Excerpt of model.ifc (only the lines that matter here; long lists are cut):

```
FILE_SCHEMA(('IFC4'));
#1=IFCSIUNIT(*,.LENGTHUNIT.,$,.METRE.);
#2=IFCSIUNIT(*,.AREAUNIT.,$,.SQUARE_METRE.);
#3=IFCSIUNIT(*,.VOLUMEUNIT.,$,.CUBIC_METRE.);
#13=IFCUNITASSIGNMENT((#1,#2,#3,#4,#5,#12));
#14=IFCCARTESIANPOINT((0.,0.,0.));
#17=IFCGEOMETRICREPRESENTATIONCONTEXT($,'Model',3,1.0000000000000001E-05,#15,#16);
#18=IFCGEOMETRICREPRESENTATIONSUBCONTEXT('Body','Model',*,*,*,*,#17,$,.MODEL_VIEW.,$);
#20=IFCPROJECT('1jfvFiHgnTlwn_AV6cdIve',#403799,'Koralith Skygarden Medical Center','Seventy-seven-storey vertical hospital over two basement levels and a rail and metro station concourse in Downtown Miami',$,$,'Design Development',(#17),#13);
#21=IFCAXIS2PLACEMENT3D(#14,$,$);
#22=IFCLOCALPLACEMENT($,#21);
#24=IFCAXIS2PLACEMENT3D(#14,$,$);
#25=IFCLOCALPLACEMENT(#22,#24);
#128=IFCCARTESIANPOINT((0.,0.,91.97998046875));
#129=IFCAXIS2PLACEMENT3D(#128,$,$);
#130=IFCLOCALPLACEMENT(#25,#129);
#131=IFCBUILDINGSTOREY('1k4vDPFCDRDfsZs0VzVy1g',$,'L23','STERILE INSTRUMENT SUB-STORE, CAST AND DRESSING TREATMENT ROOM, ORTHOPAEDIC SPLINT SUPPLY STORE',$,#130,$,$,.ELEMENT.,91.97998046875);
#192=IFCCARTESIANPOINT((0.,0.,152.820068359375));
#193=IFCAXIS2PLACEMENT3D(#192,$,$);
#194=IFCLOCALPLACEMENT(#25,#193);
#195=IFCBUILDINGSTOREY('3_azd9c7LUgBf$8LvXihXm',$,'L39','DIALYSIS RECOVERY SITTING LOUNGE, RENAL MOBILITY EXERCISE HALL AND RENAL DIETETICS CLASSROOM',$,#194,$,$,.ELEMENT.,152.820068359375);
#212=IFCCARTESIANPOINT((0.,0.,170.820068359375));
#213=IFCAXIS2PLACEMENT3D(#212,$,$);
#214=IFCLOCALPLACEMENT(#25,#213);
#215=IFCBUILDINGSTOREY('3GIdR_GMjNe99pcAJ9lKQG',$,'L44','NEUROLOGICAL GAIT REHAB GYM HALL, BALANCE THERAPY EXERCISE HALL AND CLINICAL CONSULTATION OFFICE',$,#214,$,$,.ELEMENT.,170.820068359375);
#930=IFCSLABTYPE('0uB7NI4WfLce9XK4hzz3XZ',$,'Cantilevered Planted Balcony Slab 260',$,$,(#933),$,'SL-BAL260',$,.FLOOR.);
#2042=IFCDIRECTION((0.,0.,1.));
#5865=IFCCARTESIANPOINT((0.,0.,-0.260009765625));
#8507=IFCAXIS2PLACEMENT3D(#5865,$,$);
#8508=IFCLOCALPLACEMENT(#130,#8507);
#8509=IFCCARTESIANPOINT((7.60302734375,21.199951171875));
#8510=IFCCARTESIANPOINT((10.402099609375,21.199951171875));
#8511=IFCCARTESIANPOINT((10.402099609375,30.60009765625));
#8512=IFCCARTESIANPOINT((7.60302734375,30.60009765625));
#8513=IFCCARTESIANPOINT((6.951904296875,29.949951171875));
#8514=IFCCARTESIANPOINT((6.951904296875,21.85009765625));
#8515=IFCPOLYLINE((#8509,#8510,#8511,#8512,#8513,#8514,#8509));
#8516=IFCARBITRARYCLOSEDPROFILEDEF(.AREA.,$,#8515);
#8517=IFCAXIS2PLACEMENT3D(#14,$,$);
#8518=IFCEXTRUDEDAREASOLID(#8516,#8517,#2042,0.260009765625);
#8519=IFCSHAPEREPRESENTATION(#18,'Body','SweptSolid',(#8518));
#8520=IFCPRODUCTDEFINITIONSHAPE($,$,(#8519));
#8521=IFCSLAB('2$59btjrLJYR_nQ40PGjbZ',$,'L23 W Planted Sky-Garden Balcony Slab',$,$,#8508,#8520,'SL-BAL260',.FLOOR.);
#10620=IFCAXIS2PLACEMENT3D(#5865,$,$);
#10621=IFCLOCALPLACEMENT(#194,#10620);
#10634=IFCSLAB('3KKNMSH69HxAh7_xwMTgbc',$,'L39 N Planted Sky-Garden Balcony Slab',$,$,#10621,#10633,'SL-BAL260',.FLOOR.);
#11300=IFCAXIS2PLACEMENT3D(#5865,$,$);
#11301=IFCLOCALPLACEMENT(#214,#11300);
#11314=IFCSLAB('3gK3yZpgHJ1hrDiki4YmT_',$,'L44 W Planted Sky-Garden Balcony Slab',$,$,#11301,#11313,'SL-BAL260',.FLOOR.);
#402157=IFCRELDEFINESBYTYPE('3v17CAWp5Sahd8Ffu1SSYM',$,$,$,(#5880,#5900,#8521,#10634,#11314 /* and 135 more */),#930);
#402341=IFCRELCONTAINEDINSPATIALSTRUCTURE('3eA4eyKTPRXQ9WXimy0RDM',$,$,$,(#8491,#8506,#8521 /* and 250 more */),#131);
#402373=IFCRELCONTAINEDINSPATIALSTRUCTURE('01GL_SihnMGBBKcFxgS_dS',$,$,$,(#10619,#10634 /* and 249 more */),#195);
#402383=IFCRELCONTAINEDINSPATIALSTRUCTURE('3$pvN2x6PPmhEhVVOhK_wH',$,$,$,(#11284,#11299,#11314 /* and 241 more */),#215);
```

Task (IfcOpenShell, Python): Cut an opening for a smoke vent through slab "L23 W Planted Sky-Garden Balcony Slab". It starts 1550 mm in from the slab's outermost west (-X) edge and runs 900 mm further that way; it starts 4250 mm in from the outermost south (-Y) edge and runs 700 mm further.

```python
import numpy as np
import ifcopenshell
import ifcopenshell.api.feature
import ifcopenshell.api.geometry
import ifcopenshell.api.root
import ifcopenshell.geom
import ifcopenshell.util.placement
import ifcopenshell.util.representation
import ifcopenshell.util.shape
import ifcopenshell.util.unit

model = ifcopenshell.open("model.ifc")
unit_scale = ifcopenshell.util.unit.calculate_unit_scale(model)
settings = ifcopenshell.geom.settings()


def volume(element):
    """Net volume in cubic metres, openings subtracted."""
    shape = ifcopenshell.geom.create_shape(settings, element)
    return ifcopenshell.util.shape.get_volume(shape.geometry)


slab = model.by_id(8521)
before = volume(slab)

# Extent in the slab's own axes, in metres. The edges named are its -X and -Y sides.
slab_shape = ifcopenshell.geom.create_shape(settings, slab)
vertices = ifcopenshell.util.shape.get_vertices(slab_shape.geometry)
x_min, y_min, bottom = vertices.min(axis=0)
top = vertices[:, 2].max()

opening = ifcopenshell.api.root.create_entity(model, ifc_class="IfcOpeningElement", name="Smoke vent opening", predefined_type="OPENING")
context = ifcopenshell.util.representation.get_context(model, "Model", "Body", "MODEL_VIEW")
width, depth = 0.9, 0.7
outline = [(0.0, 0.0), (width, 0.0), (width, depth), (0.0, depth), (0.0, 0.0)]
# Overshoot both faces by 50 mm so the cut is clean.
shape = ifcopenshell.api.geometry.add_slab_representation(
    model, context=context, depth=top - bottom + 0.1, polyline=outline
)
ifcopenshell.api.geometry.assign_representation(model, product=opening, representation=shape)

matrix = ifcopenshell.util.placement.get_local_placement(slab.ObjectPlacement)
matrix[:, 3] = matrix @ np.append(np.array([x_min + 1.55, y_min + 4.25, bottom - 0.05]) / unit_scale, 1.0)
ifcopenshell.api.geometry.edit_object_placement(model, product=opening, matrix=matrix, is_si=False)
ifcopenshell.api.feature.add_feature(model, feature=opening, element=slab)

after = volume(slab)

print(f"slab volume {before:.3f} -> {after:.3f} m3")

model.write("model_updated.ifc")
```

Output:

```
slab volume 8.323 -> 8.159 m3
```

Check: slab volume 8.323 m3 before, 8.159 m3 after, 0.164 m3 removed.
